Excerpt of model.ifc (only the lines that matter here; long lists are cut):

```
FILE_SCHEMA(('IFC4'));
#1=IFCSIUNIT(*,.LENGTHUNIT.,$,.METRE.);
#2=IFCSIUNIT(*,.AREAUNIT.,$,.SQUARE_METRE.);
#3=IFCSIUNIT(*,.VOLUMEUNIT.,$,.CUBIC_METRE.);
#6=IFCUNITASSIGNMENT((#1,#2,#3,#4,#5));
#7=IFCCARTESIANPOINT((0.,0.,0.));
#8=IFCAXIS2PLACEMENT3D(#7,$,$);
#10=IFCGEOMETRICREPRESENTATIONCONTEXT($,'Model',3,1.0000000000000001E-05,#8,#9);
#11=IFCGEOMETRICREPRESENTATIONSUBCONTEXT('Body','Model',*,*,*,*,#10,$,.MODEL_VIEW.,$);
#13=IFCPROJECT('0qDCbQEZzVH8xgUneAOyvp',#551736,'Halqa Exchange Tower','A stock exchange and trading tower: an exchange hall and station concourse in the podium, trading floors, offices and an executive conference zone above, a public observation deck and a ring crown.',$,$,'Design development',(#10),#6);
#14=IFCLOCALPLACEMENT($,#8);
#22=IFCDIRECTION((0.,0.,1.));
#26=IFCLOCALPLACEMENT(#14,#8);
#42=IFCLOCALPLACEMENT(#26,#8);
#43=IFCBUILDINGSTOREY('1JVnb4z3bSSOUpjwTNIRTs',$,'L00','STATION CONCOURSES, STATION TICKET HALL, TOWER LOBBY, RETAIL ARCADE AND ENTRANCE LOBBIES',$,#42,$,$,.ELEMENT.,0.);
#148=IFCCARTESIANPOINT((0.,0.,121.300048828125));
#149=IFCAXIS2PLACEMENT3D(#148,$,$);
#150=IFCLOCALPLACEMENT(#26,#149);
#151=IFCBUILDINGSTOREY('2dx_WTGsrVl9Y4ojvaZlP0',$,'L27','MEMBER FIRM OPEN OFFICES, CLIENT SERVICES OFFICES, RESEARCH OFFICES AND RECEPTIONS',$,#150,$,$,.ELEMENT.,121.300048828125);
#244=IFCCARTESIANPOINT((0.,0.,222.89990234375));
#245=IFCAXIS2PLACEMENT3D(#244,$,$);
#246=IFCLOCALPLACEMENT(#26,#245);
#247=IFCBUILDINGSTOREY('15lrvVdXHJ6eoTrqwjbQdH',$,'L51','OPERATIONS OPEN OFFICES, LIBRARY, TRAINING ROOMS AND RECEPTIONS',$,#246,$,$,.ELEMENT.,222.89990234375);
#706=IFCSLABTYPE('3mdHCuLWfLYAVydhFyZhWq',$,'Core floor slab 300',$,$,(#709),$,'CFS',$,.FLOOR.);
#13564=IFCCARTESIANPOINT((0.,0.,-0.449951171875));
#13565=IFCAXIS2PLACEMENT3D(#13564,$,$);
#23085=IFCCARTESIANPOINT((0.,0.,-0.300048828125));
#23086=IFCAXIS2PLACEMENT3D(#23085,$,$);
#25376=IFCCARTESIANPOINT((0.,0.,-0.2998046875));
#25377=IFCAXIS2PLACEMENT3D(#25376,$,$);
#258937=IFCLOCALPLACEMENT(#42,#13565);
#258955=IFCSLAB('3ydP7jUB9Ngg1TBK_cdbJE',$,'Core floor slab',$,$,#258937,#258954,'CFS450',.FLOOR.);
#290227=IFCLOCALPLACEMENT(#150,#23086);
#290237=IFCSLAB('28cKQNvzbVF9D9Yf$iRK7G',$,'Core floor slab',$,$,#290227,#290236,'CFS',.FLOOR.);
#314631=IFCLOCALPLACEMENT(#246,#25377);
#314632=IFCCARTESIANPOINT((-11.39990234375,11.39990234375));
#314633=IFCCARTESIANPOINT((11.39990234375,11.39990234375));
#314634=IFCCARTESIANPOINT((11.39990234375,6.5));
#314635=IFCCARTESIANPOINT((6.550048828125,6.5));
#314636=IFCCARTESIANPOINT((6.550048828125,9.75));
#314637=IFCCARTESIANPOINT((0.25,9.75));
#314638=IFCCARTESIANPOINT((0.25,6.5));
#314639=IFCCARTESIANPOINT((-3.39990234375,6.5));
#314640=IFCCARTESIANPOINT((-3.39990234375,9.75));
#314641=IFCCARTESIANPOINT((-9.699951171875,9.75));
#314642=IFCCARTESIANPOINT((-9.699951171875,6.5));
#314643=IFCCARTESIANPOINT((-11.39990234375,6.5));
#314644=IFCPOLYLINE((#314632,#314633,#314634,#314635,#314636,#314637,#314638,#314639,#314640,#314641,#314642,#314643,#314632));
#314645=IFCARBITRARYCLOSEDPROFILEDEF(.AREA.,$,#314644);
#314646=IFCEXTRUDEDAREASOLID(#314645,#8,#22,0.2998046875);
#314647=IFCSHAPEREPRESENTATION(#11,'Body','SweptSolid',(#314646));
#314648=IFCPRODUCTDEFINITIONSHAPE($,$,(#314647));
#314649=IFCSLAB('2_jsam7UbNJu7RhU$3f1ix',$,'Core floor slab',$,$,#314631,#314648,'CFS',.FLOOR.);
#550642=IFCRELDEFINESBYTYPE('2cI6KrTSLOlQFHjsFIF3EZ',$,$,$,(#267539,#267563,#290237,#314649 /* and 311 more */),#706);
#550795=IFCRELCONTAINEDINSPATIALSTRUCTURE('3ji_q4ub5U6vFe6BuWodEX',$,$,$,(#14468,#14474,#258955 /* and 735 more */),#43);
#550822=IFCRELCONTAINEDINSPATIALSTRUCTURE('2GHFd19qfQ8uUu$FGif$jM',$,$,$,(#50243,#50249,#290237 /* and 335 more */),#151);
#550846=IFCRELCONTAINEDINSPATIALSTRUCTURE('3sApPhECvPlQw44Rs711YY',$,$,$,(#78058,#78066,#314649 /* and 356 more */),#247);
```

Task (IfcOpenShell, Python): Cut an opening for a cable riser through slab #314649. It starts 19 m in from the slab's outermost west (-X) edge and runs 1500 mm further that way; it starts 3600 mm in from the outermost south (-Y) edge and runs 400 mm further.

```python
import numpy as np
import ifcopenshell
import ifcopenshell.api.feature
import ifcopenshell.api.geometry
import ifcopenshell.api.root
import ifcopenshell.geom
import ifcopenshell.util.placement
import ifcopenshell.util.representation
import ifcopenshell.util.shape
import ifcopenshell.util.unit

model = ifcopenshell.open("model.ifc")
unit_scale = ifcopenshell.util.unit.calculate_unit_scale(model)
settings = ifcopenshell.geom.settings()


def volume(element):
    """Net volume in cubic metres, openings subtracted."""
    shape = ifcopenshell.geom.create_shape(settings, element)
    return ifcopenshell.util.shape.get_volume(shape.geometry)


slab = model.by_guid("2_jsam7UbNJu7RhU$3f1ix")
before = volume(slab)

# Extent in the slab's own axes, in metres. The edges named are its -X and -Y sides.
slab_shape = ifcopenshell.geom.create_shape(settings, slab)
vertices = ifcopenshell.util.shape.get_vertices(slab_shape.geometry)
x_min, y_min, bottom = vertices.min(axis=0)
top = vertices[:, 2].max()

opening = ifcopenshell.api.root.create_entity(model, ifc_class="IfcOpeningElement", name="Cable riser opening", predefined_type="OPENING")
context = ifcopenshell.util.representation.get_context(model, "Model", "Body", "MODEL_VIEW")
width, depth = 1.5, 0.4
outline = [(0.0, 0.0), (width, 0.0), (width, depth), (0.0, depth), (0.0, 0.0)]
# Overshoot both faces by 50 mm so the cut is clean.
shape = ifcopenshell.api.geometry.add_slab_representation(
    model, context=context, depth=top - bottom + 0.1, polyline=outline
)
ifcopenshell.api.geometry.assign_representation(model, product=opening, representation=shape)

matrix = ifcopenshell.util.placement.get_local_placement(slab.ObjectPlacement)
matrix[:, 3] = matrix @ np.append(np.array([x_min + 19, y_min + 3.6, bottom - 0.05]) / unit_scale, 1.0)
ifcopenshell.api.geometry.edit_object_placement(model, product=opening, matrix=matrix, is_si=False)
ifcopenshell.api.feature.add_feature(model, feature=opening, element=slab)

after = volume(slab)

print(f"slab volume {before:.3f} -> {after:.3f} m3")

model.write("model-out.ifc")
```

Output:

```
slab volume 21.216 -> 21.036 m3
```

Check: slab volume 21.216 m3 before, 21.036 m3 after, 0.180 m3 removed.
